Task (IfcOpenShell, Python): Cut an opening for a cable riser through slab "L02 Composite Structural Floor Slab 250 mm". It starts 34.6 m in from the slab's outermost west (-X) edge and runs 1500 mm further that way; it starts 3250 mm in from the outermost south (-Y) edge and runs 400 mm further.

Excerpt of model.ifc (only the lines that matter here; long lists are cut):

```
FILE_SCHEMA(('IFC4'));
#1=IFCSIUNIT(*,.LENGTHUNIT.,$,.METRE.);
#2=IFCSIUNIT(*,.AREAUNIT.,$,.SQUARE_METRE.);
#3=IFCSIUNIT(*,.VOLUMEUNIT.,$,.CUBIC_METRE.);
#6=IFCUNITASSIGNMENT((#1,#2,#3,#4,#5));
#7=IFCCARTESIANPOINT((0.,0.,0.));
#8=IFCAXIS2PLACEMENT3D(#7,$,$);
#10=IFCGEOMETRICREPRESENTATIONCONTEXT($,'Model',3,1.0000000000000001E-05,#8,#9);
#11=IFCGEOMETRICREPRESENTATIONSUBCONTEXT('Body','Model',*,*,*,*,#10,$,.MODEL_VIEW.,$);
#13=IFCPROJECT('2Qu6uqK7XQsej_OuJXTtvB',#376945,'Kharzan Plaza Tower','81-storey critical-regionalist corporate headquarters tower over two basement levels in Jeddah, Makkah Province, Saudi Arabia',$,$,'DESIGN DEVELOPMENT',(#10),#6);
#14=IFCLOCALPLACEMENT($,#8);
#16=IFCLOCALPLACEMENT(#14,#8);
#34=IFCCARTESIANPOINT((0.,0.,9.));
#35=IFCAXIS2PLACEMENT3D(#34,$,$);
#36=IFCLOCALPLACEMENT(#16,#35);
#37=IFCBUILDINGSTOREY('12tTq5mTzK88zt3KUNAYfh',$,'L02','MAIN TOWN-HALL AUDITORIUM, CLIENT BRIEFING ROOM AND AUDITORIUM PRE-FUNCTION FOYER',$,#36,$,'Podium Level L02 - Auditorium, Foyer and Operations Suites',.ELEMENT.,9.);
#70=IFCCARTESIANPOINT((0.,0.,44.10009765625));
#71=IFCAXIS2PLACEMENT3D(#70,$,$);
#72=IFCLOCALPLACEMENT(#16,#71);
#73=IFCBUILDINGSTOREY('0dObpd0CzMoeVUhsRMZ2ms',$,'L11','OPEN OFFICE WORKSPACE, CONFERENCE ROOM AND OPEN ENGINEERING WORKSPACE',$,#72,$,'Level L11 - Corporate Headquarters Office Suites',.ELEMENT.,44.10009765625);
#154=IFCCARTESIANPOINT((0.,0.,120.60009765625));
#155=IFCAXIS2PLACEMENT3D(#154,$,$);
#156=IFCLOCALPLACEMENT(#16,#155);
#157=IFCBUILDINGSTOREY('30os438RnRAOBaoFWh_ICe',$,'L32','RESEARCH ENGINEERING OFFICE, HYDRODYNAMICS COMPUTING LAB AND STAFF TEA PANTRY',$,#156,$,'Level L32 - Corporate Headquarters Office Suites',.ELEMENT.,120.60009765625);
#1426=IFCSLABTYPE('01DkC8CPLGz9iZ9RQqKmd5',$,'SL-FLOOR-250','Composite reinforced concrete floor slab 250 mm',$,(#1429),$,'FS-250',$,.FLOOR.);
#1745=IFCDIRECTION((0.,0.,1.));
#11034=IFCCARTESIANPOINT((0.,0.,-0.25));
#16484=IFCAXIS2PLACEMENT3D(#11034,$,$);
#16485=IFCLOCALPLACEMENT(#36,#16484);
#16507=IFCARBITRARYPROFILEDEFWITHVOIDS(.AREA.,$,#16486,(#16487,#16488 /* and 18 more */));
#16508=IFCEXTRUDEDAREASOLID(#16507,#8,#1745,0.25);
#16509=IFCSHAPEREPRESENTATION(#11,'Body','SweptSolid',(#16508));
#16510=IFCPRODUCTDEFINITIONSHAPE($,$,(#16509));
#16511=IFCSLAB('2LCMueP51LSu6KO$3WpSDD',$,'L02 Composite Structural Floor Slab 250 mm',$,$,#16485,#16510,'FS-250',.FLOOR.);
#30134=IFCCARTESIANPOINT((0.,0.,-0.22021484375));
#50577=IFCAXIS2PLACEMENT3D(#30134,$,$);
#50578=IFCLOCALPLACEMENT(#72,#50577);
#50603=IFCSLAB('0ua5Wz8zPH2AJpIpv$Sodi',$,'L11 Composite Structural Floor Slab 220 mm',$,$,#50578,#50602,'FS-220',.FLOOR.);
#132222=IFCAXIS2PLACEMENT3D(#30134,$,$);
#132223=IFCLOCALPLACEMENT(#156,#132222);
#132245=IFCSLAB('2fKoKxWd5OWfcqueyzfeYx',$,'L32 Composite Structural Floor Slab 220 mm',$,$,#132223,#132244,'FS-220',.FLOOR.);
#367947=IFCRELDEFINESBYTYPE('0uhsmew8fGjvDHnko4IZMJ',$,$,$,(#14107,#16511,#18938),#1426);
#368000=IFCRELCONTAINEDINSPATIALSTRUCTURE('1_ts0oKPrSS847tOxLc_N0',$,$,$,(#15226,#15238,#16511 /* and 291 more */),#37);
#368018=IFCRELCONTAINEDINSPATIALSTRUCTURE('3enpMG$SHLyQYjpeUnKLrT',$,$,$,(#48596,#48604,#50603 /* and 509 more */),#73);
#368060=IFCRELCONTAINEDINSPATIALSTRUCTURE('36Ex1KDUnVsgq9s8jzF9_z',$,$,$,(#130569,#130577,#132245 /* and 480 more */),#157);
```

```python
import numpy as np
import ifcopenshell
import ifcopenshell.api.feature
import ifcopenshell.api.geometry
import ifcopenshell.api.root
import ifcopenshell.geom
import ifcopenshell.util.placement
import ifcopenshell.util.representation
import ifcopenshell.util.shape
import ifcopenshell.util.unit

model = ifcopenshell.open("model.ifc")
unit_scale = ifcopenshell.util.unit.calculate_unit_scale(model)
settings = ifcopenshell.geom.settings()


def volume(element):
    """Net volume in cubic metres, openings subtracted."""
    shape = ifcopenshell.geom.create_shape(settings, element)
    return ifcopenshell.util.shape.get_volume(shape.geometry)


slab = model.by_guid("2LCMueP51LSu6KO$3WpSDD")
before = volume(slab)

# Extent in the slab's own axes, in metres. The edges named are its -X and -Y sides.
slab_shape = ifcopenshell.geom.create_shape(settings, slab)
vertices = ifcopenshell.util.shape.get_vertices(slab_shape.geometry)
x_min, y_min, bottom = vertices.min(axis=0)
top = vertices[:, 2].max()

opening = ifcopenshell.api.root.create_entity(model, ifc_class="IfcOpeningElement", name="Cable riser opening", predefined_type="OPENING")
context = ifcopenshell.util.representation.get_context(model, "Model", "Body", "MODEL_VIEW")
width, depth = 1.5, 0.4
outline = [(0.0, 0.0), (width, 0.0), (width, depth), (0.0, depth), (0.0, 0.0)]
# Overshoot both faces by 50 mm so the cut is clean.
shape = ifcopenshell.api.geometry.add_slab_representation(
    model, context=context, depth=top - bottom + 0.1, polyline=outline
)
ifcopenshell.api.geometry.assign_representation(model, product=opening, representation=shape)

matrix = ifcopenshell.util.placement.get_local_placement(slab.ObjectPlacement)
matrix[:, 3] = matrix @ np.append(np.array([x_min + 34.6, y_min + 3.25, bottom - 0.05]) / unit_scale, 1.0)
ifcopenshell.api.geometry.edit_object_placement(model, product=opening, matrix=matrix, is_si=False)
ifcopenshell.api.feature.add_feature(model, feature=opening, element=slab)

after = volume(slab)

print(f"slab volume {before:.3f} -> {after:.3f} m3")

model.write("model_updated.ifc")
```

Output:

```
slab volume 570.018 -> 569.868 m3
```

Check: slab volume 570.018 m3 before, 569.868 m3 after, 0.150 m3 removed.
